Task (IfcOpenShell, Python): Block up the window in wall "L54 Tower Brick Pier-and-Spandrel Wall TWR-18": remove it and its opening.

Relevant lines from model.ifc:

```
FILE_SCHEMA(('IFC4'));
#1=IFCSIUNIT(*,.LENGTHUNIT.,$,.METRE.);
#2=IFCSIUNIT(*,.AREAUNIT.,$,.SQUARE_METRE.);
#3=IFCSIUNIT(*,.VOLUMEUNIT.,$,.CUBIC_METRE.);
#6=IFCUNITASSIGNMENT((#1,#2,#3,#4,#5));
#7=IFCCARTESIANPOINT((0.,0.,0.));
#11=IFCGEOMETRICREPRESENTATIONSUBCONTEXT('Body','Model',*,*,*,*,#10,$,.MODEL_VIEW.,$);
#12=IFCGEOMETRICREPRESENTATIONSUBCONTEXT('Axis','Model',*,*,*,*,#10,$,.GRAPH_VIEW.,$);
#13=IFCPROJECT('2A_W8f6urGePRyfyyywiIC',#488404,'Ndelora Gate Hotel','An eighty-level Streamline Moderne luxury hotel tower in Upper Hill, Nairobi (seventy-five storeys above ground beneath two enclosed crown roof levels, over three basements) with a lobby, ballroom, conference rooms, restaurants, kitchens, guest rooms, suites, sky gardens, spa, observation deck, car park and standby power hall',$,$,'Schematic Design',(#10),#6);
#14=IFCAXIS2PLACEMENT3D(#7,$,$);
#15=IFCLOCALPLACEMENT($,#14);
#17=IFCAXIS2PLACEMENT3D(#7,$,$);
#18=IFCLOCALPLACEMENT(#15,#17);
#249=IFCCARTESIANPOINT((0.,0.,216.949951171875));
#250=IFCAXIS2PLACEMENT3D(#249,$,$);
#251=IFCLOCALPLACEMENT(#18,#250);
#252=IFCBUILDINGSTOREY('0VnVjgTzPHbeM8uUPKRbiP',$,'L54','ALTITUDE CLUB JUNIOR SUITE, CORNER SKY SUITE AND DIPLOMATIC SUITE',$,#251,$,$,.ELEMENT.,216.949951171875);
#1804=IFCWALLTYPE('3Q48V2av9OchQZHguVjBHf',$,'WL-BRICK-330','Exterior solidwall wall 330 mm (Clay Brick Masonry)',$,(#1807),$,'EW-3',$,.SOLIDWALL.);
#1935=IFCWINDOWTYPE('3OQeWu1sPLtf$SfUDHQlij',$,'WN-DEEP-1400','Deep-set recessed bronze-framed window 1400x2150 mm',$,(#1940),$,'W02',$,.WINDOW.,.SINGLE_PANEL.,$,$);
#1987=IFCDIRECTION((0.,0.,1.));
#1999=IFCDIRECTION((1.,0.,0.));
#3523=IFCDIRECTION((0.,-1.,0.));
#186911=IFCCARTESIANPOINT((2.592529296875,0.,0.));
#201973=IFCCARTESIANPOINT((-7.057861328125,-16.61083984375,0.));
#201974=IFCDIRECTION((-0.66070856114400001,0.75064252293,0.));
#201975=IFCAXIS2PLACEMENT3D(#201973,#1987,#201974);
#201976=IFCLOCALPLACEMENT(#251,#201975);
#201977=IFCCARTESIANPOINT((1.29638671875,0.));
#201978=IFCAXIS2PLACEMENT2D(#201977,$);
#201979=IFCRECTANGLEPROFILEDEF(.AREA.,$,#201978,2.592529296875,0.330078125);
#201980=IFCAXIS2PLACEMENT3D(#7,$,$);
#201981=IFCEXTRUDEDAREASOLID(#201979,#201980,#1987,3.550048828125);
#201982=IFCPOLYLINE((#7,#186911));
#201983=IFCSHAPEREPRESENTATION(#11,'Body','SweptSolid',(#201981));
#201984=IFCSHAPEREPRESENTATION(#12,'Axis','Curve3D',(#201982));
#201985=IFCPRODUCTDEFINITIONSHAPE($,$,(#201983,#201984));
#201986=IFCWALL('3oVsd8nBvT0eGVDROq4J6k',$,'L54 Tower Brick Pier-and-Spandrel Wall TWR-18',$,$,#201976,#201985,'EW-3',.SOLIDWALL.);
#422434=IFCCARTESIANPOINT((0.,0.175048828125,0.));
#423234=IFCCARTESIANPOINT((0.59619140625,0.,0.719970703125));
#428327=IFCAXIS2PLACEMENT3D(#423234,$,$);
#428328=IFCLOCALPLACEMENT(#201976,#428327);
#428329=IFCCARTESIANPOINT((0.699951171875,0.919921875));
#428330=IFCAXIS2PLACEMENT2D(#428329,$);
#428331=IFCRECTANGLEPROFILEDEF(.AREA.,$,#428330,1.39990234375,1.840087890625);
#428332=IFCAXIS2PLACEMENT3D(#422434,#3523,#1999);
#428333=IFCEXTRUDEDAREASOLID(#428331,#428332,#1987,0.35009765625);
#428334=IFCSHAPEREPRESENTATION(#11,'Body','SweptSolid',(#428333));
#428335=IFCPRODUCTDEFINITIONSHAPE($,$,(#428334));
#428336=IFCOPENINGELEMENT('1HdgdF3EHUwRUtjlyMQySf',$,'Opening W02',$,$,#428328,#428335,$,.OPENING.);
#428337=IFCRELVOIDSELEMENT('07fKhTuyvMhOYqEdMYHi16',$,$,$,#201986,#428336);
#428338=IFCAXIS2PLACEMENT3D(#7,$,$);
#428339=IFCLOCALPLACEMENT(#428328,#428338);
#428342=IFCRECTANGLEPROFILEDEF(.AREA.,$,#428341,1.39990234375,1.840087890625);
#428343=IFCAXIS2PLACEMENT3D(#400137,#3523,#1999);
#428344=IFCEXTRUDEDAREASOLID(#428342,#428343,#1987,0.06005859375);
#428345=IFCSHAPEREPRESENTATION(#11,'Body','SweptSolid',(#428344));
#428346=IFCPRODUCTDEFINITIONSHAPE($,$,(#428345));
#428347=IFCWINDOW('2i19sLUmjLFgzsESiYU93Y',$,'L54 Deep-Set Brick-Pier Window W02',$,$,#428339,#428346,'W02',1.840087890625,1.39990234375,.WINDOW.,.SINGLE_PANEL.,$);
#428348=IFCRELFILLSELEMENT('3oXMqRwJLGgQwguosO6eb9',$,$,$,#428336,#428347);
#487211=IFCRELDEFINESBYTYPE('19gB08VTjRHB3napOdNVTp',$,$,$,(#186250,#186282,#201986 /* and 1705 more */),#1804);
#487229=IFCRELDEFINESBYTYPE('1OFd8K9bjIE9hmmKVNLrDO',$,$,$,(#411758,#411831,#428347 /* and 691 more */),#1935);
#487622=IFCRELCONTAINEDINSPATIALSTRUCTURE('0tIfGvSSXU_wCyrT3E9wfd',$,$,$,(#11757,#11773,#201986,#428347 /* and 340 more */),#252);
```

```python
import ifcopenshell
import ifcopenshell.api.feature
import ifcopenshell.api.root
import ifcopenshell.geom
import ifcopenshell.util.shape

model = ifcopenshell.open("model.ifc")
settings = ifcopenshell.geom.settings()


def volume(element):
    """Net volume in cubic metres, openings subtracted."""
    shape = ifcopenshell.geom.create_shape(settings, element)
    return ifcopenshell.util.shape.get_volume(shape.geometry)


window = model.by_id(428347)
opening = window.FillsVoids[0].RelatingOpeningElement
wall = opening.VoidsElements[0].RelatingBuildingElement
before = volume(wall)

ifcopenshell.api.root.remove_product(model, product=window)
ifcopenshell.api.feature.remove_feature(model, feature=opening)

after = volume(wall)

print(f"wall volume {before:.3f} -> {after:.3f} m3")

model.write("model_updated.ifc")
```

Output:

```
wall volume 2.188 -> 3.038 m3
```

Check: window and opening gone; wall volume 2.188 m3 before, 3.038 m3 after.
